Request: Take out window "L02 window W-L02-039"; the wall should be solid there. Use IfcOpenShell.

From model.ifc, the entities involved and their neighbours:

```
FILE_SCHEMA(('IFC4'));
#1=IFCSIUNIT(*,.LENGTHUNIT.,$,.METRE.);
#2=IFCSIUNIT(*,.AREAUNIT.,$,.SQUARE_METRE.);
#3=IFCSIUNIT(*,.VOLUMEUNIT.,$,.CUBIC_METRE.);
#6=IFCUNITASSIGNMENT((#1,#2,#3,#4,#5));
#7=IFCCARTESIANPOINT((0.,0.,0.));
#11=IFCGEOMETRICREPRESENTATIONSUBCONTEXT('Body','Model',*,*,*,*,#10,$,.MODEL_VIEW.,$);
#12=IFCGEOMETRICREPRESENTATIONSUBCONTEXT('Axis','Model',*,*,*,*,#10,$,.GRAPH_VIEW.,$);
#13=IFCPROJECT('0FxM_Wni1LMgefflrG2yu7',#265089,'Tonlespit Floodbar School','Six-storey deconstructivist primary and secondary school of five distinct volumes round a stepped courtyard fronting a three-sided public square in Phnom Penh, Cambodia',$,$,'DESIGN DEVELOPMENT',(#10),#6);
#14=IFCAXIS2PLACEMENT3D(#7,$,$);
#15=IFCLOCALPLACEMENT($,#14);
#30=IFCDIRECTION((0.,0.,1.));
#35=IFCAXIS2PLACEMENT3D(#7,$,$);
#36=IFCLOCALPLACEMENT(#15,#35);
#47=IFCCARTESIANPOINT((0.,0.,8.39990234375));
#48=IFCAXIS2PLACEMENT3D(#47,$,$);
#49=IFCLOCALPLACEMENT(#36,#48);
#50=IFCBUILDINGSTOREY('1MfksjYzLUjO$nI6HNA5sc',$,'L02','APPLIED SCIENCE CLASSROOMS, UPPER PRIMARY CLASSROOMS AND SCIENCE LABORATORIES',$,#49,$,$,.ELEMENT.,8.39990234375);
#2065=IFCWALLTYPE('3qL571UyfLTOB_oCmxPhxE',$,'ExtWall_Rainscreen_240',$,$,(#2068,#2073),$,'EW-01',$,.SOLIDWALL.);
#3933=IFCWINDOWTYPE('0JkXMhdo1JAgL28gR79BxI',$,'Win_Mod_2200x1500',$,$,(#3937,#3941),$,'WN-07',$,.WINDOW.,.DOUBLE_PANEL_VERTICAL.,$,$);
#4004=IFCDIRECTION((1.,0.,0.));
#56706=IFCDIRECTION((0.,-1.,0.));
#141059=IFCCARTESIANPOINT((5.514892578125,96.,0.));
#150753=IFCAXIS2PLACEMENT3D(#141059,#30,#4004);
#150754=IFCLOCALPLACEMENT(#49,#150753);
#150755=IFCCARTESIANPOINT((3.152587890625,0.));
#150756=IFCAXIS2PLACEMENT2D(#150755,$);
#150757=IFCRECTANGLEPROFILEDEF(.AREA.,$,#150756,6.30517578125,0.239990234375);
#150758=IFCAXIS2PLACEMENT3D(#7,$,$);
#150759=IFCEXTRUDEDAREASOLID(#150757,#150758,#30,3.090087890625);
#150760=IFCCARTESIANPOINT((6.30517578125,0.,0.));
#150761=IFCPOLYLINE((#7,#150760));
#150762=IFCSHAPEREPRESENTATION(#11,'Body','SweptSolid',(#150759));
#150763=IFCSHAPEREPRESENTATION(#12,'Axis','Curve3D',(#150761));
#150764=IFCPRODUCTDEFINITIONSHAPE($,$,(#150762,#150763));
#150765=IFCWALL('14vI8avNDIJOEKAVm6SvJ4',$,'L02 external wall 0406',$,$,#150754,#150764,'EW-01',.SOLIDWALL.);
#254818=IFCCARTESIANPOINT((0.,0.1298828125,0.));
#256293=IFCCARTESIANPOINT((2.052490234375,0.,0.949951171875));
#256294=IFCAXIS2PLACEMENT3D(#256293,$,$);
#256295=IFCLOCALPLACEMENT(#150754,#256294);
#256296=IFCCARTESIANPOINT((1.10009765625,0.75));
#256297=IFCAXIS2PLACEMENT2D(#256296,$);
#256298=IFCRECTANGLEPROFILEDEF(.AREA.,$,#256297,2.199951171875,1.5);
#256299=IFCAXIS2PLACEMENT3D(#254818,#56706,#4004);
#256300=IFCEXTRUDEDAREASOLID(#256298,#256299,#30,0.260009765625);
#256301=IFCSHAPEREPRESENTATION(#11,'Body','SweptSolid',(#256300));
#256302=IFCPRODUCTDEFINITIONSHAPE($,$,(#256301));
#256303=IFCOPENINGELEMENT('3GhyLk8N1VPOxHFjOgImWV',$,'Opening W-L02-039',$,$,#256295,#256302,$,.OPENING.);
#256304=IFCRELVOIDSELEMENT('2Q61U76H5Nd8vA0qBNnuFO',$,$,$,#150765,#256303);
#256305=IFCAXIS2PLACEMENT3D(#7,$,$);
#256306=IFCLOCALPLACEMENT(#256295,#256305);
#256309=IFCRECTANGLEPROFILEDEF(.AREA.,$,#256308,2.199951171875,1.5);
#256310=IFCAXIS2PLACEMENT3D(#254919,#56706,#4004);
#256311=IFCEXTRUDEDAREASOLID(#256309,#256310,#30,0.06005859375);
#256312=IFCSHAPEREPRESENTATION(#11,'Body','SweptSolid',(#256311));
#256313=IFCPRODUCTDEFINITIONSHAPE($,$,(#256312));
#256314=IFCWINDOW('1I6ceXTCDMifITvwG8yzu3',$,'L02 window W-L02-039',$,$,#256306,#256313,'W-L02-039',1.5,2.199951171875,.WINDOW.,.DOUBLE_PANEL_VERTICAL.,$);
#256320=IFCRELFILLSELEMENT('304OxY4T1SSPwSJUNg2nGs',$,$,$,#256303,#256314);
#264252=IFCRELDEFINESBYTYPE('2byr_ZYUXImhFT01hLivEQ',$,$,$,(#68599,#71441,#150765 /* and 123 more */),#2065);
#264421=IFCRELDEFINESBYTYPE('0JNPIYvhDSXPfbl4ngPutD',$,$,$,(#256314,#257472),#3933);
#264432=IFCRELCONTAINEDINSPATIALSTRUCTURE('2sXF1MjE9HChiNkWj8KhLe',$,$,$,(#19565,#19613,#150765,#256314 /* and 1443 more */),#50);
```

```python
import ifcopenshell
import ifcopenshell.api.feature
import ifcopenshell.api.root
import ifcopenshell.geom
import ifcopenshell.util.shape

model = ifcopenshell.open("model.ifc")
settings = ifcopenshell.geom.settings()


def volume(element):
    """Net volume in cubic metres, openings subtracted."""
    shape = ifcopenshell.geom.create_shape(settings, element)
    return ifcopenshell.util.shape.get_volume(shape.geometry)


window = model.by_guid("1I6ceXTCDMifITvwG8yzu3")
opening = window.FillsVoids[0].RelatingOpeningElement
wall = opening.VoidsElements[0].RelatingBuildingElement
before = volume(wall)

ifcopenshell.api.root.remove_product(model, product=window)
ifcopenshell.api.feature.remove_feature(model, feature=opening)

after = volume(wall)

print(f"wall volume {before:.3f} -> {after:.3f} m3")

model.write("model_edited.ifc")
```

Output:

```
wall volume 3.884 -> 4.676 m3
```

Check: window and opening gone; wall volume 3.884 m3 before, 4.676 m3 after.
